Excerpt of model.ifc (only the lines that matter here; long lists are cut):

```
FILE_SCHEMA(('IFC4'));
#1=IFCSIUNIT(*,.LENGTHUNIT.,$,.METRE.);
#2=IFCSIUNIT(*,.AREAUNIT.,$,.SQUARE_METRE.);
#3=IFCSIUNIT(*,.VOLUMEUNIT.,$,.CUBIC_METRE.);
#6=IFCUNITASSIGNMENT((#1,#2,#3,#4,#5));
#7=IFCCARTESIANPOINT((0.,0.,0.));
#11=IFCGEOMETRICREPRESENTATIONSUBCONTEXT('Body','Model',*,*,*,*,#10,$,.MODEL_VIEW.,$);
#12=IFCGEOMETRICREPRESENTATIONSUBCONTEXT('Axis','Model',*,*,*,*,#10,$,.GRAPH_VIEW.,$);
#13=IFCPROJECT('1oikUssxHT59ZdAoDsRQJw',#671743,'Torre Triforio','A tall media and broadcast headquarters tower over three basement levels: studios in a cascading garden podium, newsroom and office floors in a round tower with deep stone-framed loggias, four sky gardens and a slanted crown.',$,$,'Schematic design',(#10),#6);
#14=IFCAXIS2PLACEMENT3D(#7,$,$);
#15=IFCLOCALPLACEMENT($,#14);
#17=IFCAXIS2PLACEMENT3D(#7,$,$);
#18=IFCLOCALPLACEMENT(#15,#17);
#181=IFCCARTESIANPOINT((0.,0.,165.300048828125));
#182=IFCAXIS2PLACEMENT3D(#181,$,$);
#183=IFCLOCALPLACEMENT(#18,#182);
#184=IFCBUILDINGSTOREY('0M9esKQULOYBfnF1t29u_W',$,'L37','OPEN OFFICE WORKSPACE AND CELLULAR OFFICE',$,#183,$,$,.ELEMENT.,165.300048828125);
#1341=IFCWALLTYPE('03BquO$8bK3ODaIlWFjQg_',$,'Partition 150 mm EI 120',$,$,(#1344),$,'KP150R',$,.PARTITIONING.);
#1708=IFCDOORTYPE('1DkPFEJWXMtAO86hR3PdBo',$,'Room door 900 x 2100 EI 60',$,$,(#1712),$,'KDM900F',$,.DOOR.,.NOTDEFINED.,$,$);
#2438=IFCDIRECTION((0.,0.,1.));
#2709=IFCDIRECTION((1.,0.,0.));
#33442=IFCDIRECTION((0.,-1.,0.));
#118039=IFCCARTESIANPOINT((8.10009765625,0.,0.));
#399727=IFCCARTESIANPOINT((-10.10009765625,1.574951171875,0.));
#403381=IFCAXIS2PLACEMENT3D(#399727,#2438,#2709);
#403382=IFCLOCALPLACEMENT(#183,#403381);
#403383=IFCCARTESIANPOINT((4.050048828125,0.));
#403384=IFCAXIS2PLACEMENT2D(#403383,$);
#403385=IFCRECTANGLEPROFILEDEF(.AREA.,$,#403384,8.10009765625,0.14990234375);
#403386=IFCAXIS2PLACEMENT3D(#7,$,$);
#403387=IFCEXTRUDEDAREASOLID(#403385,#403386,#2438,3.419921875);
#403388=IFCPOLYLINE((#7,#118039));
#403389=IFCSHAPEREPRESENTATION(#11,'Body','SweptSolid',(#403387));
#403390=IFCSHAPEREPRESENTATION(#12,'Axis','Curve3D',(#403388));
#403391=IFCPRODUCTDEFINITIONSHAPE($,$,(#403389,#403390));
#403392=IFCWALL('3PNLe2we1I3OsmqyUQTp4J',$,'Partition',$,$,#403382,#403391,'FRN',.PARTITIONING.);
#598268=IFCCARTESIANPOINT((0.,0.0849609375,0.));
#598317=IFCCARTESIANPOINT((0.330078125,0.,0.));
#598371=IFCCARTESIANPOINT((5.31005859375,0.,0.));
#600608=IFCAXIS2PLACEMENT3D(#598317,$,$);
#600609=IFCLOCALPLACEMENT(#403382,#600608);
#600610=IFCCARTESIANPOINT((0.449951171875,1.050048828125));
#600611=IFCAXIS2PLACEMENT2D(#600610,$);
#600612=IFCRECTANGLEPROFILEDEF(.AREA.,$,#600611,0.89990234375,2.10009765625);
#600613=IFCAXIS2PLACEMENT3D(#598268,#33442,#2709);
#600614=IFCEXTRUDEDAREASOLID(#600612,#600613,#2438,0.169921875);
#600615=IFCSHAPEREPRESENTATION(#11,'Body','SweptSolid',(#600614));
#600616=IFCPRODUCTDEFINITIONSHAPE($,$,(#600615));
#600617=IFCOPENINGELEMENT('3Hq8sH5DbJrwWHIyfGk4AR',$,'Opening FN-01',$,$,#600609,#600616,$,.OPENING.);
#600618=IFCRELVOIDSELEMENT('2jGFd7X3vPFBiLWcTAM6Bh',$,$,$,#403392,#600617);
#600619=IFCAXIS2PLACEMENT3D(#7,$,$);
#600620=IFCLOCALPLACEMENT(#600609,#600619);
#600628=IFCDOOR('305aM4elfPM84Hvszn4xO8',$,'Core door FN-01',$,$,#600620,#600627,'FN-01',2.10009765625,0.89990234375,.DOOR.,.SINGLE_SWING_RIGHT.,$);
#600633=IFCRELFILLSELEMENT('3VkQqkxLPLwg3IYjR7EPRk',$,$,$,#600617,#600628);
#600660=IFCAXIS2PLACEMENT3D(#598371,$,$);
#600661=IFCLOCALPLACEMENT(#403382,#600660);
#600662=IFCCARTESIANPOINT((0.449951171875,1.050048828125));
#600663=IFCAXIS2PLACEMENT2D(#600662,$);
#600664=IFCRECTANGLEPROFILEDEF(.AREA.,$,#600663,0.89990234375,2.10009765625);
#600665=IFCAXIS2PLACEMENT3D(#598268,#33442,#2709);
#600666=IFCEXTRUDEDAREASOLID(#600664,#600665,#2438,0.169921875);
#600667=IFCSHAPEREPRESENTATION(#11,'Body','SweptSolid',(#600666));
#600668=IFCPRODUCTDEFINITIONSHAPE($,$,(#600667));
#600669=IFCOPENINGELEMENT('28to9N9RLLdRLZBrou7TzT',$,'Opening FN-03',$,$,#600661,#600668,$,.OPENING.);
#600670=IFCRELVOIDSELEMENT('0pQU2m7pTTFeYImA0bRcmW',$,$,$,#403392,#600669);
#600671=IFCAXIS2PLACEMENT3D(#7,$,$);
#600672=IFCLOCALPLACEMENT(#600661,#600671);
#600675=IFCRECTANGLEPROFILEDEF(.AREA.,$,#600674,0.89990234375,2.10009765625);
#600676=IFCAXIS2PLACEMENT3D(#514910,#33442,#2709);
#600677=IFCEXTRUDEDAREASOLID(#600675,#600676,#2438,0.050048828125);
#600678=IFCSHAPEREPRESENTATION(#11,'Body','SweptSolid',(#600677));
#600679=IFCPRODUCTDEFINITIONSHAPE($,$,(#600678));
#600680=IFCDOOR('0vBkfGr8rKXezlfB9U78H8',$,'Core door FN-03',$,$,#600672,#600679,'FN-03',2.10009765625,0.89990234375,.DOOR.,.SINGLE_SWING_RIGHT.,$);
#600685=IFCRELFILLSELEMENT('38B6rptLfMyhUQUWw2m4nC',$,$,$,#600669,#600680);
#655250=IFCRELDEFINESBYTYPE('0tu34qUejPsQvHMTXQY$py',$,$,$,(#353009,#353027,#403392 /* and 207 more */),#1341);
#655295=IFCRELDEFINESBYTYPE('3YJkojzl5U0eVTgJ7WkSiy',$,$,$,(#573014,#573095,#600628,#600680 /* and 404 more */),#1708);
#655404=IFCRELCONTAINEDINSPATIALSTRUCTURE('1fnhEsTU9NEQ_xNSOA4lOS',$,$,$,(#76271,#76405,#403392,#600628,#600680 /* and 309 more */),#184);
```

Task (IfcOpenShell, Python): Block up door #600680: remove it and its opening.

```python
import ifcopenshell
import ifcopenshell.api.feature
import ifcopenshell.api.root
import ifcopenshell.geom
import ifcopenshell.util.shape

model = ifcopenshell.open("model.ifc")
settings = ifcopenshell.geom.settings()


def volume(element):
    """Net volume in cubic metres, openings subtracted."""
    shape = ifcopenshell.geom.create_shape(settings, element)
    return ifcopenshell.util.shape.get_volume(shape.geometry)


door = model.by_guid("0vBkfGr8rKXezlfB9U78H8")
opening = door.FillsVoids[0].RelatingOpeningElement
wall = opening.VoidsElements[0].RelatingBuildingElement
before = volume(wall)

ifcopenshell.api.root.remove_product(model, product=door)
ifcopenshell.api.feature.remove_feature(model, feature=opening)

after = volume(wall)

print(f"wall volume {before:.3f} -> {after:.3f} m3")

model.write("model_rev.ifc")
```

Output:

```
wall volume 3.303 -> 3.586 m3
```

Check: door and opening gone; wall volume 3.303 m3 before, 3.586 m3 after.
